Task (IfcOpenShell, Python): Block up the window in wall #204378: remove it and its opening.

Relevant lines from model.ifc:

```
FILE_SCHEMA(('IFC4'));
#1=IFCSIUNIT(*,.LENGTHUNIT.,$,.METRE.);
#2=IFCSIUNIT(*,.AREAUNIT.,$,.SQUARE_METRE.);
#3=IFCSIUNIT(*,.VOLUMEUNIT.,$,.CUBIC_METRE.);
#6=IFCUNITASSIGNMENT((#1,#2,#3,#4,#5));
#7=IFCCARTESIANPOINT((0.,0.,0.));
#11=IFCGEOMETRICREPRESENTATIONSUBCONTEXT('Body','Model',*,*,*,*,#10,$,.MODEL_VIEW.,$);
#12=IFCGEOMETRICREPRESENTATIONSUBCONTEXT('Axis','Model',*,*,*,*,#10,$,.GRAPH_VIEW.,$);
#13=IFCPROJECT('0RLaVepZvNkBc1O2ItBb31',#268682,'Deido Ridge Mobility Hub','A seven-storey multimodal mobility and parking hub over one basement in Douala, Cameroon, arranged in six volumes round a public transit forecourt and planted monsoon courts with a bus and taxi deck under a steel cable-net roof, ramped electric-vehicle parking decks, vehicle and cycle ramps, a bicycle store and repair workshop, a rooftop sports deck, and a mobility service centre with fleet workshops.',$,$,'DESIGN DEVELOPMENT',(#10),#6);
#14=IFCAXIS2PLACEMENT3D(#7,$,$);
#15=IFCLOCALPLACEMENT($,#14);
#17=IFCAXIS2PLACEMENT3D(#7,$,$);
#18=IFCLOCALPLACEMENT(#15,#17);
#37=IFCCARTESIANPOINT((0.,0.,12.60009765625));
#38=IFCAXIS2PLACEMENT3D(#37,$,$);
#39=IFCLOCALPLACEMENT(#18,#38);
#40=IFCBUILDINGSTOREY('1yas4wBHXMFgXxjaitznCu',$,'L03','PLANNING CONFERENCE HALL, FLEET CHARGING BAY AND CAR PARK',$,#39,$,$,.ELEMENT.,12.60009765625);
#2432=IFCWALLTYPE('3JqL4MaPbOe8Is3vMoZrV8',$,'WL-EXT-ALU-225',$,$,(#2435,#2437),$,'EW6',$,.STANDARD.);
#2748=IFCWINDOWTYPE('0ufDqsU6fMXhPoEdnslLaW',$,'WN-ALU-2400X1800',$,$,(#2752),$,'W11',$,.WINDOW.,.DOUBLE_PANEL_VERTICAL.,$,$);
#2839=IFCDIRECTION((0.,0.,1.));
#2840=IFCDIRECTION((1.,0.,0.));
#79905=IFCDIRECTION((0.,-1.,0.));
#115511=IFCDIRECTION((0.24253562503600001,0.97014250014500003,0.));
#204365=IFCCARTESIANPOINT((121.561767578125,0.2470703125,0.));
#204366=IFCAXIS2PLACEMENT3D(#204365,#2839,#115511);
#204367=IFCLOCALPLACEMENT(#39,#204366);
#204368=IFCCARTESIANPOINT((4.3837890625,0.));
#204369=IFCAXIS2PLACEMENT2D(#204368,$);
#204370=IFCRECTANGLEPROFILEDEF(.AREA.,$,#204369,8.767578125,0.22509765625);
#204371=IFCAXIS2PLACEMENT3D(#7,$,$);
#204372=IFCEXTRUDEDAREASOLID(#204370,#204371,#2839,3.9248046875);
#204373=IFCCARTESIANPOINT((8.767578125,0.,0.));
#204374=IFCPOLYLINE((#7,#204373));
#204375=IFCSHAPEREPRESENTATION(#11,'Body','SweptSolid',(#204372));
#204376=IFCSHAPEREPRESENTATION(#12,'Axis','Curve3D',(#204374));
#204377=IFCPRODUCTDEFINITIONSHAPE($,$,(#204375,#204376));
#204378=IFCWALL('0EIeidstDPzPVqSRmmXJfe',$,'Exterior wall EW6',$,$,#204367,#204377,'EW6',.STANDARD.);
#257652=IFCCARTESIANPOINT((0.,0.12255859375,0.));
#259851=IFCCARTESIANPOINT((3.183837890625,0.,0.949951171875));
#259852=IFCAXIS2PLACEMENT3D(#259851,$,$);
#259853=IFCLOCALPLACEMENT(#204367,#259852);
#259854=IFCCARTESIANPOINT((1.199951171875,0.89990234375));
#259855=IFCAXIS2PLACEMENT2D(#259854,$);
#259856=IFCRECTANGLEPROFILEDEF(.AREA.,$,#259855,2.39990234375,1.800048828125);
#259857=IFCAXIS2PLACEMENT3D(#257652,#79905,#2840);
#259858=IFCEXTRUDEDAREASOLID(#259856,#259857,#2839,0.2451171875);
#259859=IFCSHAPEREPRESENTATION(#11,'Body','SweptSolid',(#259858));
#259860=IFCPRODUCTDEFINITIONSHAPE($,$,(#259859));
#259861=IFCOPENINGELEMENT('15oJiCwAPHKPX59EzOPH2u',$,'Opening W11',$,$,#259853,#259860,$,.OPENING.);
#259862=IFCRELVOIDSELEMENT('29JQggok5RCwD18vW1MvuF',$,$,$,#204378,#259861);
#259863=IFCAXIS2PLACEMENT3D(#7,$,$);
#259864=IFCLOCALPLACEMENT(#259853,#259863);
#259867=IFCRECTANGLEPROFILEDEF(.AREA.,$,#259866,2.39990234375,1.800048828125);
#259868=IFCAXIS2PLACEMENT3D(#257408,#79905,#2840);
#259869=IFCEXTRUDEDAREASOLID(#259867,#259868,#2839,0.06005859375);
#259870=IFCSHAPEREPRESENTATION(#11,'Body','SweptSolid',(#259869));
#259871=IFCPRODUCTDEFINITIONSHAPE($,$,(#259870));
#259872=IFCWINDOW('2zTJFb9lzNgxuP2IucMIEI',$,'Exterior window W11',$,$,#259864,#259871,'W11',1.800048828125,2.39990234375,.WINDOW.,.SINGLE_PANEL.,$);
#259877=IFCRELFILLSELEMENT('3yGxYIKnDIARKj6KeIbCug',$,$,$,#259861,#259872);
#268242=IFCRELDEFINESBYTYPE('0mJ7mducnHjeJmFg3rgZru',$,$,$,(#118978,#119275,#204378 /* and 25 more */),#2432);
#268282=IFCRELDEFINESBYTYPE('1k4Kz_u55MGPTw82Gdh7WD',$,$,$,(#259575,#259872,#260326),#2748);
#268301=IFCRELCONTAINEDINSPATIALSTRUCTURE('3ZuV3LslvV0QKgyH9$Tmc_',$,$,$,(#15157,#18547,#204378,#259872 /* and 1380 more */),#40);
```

```python
import ifcopenshell
import ifcopenshell.api.feature
import ifcopenshell.api.root
import ifcopenshell.geom
import ifcopenshell.util.shape

model = ifcopenshell.open("model.ifc")
settings = ifcopenshell.geom.settings()


def volume(element):
    """Net volume in cubic metres, openings subtracted."""
    shape = ifcopenshell.geom.create_shape(settings, element)
    return ifcopenshell.util.shape.get_volume(shape.geometry)


window = model.by_guid("2zTJFb9lzNgxuP2IucMIEI")
opening = window.FillsVoids[0].RelatingOpeningElement
wall = opening.VoidsElements[0].RelatingBuildingElement
before = volume(wall)

ifcopenshell.api.root.remove_product(model, product=window)
ifcopenshell.api.feature.remove_feature(model, feature=opening)

after = volume(wall)

print(f"wall volume {before:.3f} -> {after:.3f} m3")

model.write("model_edited.ifc")
```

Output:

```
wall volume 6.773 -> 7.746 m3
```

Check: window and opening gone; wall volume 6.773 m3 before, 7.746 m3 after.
